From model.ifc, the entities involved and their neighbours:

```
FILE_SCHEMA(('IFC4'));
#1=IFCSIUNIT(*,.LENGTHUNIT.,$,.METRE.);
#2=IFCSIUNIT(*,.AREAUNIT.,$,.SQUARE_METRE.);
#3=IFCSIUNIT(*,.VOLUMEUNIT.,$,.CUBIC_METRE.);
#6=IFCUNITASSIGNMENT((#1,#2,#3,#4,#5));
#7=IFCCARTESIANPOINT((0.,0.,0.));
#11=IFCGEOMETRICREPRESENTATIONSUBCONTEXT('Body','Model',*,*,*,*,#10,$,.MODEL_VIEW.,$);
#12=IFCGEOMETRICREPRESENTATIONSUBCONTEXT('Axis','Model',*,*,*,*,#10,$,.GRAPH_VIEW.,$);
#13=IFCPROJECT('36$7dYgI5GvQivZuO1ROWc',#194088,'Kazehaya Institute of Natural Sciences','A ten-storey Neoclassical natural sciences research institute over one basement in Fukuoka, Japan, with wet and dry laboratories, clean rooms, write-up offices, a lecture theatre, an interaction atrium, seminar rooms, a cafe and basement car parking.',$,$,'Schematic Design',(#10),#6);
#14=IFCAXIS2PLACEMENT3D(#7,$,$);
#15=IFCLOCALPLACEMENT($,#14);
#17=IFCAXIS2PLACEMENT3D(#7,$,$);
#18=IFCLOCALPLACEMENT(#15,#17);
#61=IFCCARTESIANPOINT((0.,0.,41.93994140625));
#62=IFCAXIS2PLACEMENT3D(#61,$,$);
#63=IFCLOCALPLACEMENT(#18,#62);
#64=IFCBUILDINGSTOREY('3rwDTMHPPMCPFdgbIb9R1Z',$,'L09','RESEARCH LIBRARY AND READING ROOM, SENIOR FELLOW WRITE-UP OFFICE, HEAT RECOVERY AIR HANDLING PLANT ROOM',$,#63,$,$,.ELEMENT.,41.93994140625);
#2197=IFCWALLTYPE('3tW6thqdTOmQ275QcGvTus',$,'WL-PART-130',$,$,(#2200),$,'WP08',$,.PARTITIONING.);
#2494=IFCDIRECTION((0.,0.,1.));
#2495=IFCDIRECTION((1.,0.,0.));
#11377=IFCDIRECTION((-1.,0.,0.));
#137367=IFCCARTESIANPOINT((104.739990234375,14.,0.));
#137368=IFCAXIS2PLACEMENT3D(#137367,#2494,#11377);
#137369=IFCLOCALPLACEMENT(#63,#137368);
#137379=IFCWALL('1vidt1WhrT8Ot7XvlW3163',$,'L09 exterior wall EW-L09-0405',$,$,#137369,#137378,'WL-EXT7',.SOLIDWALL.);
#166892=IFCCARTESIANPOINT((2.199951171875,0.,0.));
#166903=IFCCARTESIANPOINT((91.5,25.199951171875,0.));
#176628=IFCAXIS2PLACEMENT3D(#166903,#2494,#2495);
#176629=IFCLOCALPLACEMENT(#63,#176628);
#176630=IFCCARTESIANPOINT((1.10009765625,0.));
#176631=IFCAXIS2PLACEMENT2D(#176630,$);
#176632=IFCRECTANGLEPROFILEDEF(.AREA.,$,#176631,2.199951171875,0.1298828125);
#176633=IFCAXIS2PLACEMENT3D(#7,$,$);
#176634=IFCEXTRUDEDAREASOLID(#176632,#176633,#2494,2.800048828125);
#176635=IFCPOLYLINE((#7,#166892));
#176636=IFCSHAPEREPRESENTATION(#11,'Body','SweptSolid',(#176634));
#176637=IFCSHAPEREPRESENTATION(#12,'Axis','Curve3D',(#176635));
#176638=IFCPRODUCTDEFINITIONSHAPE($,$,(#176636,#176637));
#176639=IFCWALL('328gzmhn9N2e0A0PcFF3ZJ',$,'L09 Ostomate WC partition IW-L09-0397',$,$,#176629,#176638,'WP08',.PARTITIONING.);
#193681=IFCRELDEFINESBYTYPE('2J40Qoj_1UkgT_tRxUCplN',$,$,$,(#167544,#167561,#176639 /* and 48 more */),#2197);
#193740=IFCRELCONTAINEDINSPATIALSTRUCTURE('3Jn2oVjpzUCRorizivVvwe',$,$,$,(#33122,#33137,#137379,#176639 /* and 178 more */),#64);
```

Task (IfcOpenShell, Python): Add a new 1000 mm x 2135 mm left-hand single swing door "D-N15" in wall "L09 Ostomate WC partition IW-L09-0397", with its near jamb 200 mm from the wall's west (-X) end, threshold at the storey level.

```python
import numpy as np
import ifcopenshell
import ifcopenshell.api.feature
import ifcopenshell.api.geometry
import ifcopenshell.api.root
import ifcopenshell.api.spatial
import ifcopenshell.geom
import ifcopenshell.util.element
import ifcopenshell.util.placement
import ifcopenshell.util.representation
import ifcopenshell.util.shape
import ifcopenshell.util.unit

model = ifcopenshell.open("model.ifc")
unit_scale = ifcopenshell.util.unit.calculate_unit_scale(model)
settings = ifcopenshell.geom.settings()


def volume(element):
    """Net volume in cubic metres, openings subtracted."""
    shape = ifcopenshell.geom.create_shape(settings, element)
    return ifcopenshell.util.shape.get_volume(shape.geometry)


wall = model.by_guid("328gzmhn9N2e0A0PcFF3ZJ")
storey = ifcopenshell.util.element.get_container(wall, ifc_class="IfcBuildingStorey")
context = ifcopenshell.util.representation.get_context(model, "Model", "Body", "MODEL_VIEW")
before = volume(wall)

width, height, from_end, sill = 1, 2.135, 0.2, 0.0  # metres

# The wall runs along its own X axis, and the end named is its -X end.
wall_shape = ifcopenshell.geom.create_shape(settings, wall)
x, y, z = ifcopenshell.util.shape.get_vertices(wall_shape.geometry).T
start = x.min() + from_end
face, thickness = float(y.min()), float(y.max() - y.min())
wall_matrix = ifcopenshell.util.placement.get_local_placement(wall.ObjectPlacement)
level = ifcopenshell.util.placement.get_local_placement(storey.ObjectPlacement)[2, 3]


def in_wall(x, y):
    """Placement at x, y metres in the wall's axes, at sill height."""
    matrix = wall_matrix.copy()
    matrix[:, 3] = wall_matrix @ np.array([x / unit_scale, y / unit_scale, 0.0, 1.0])
    matrix[2, 3] = level + sill / unit_scale
    return matrix


# Opening: a box that overshoots both wall faces by 50 mm.
opening = ifcopenshell.api.root.create_entity(model, ifc_class="IfcOpeningElement", predefined_type="OPENING")
box = ifcopenshell.api.geometry.add_wall_representation(
    model, context=context, length=width, height=height, thickness=thickness + 0.1
)
ifcopenshell.api.geometry.assign_representation(model, product=opening, representation=box)
ifcopenshell.api.geometry.edit_object_placement(model, product=opening, matrix=in_wall(start, face - 0.05), is_si=False)
ifcopenshell.api.feature.add_feature(model, feature=opening, element=wall)

door = ifcopenshell.api.root.create_entity(model, ifc_class="IfcDoor", name="D-N15", predefined_type="DOOR")
door.OverallWidth, door.OverallHeight = width / unit_scale, height / unit_scale
door.OperationType = "SINGLE_SWING_LEFT"
body = ifcopenshell.api.geometry.add_door_representation(
    model,
    context=context,
    overall_width=door.OverallWidth,
    overall_height=door.OverallHeight,
    operation_type="SINGLE_SWING_LEFT",
    lining_properties={"LiningDepth": thickness / unit_scale, "ThresholdDepth": thickness / unit_scale},
)
ifcopenshell.api.geometry.assign_representation(model, product=door, representation=body)
ifcopenshell.api.spatial.assign_container(model, products=[door], relating_structure=storey)
ifcopenshell.api.feature.add_filling(model, opening=opening, element=door)

# The lining spans the wall, so the door starts at the wall face.
ifcopenshell.api.geometry.edit_object_placement(model, product=door, matrix=in_wall(start, face), is_si=False)

after = volume(wall)

print(f"wall volume {before:.3f} -> {after:.3f} m3")

model.write("model-out.ifc")
```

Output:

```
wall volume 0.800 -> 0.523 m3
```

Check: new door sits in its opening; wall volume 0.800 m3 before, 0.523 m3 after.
